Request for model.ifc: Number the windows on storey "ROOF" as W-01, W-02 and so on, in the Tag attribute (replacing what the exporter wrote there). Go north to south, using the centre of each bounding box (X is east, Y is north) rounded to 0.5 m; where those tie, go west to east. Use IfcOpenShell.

First a look at what the model holds.

```python
import ifcopenshell
import ifcopenshell.util.element
import ifcopenshell.util.placement

model = ifcopenshell.open("model.ifc")
print(model.schema)
storey = next(s for s in model.by_type("IfcBuildingStorey") if s.Name == "ROOF")
windows = [e for e in ifcopenshell.util.element.get_decomposition(storey) if e.is_a("IfcWindow")]
for e in sorted(windows, key=lambda e: e.id()):
    origin = ifcopenshell.util.placement.get_local_placement(e.ObjectPlacement)[:3, 3]
    print(e.id(), e.Tag, e.Name, origin.round(2) + 0.0, sep=" | ")
```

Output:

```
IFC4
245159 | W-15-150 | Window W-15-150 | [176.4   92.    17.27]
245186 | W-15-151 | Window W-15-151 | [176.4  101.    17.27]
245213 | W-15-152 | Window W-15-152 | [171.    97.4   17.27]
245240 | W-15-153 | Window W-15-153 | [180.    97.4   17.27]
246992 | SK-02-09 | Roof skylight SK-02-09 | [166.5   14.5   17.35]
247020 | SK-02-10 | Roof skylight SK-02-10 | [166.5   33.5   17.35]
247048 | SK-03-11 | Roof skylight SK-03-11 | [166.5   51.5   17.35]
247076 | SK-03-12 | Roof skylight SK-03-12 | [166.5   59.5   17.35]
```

```python
import ifcopenshell
import ifcopenshell.geom
import ifcopenshell.util.element
import ifcopenshell.util.shape

model = ifcopenshell.open("model.ifc")
settings = ifcopenshell.geom.settings()
settings.set("use-world-coords", True)


def centre(element):
    shape = ifcopenshell.geom.create_shape(settings, element)
    return ifcopenshell.util.shape.get_bbox_centroid(shape.geometry)


storey = next(s for s in model.by_type("IfcBuildingStorey") if s.Name == "ROOF")
windows = [e for e in ifcopenshell.util.element.get_decomposition(storey) if e.is_a("IfcWindow")]

# Insertion points can sit at a corner or the storey origin, so sort by the geometry (in metres).
centres = {e: centre(e) for e in windows}
windows.sort(key=lambda e: (-round(centres[e][1] / 0.5), centres[e][0]))

for i, e in enumerate(windows, start=1):
    number = f"W-{i:02d}"
    e.Tag = number
    print(e.id(), number)

model.write("model_rev.ifc")
```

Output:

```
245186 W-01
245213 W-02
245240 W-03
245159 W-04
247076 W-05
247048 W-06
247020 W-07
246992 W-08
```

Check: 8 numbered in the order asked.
